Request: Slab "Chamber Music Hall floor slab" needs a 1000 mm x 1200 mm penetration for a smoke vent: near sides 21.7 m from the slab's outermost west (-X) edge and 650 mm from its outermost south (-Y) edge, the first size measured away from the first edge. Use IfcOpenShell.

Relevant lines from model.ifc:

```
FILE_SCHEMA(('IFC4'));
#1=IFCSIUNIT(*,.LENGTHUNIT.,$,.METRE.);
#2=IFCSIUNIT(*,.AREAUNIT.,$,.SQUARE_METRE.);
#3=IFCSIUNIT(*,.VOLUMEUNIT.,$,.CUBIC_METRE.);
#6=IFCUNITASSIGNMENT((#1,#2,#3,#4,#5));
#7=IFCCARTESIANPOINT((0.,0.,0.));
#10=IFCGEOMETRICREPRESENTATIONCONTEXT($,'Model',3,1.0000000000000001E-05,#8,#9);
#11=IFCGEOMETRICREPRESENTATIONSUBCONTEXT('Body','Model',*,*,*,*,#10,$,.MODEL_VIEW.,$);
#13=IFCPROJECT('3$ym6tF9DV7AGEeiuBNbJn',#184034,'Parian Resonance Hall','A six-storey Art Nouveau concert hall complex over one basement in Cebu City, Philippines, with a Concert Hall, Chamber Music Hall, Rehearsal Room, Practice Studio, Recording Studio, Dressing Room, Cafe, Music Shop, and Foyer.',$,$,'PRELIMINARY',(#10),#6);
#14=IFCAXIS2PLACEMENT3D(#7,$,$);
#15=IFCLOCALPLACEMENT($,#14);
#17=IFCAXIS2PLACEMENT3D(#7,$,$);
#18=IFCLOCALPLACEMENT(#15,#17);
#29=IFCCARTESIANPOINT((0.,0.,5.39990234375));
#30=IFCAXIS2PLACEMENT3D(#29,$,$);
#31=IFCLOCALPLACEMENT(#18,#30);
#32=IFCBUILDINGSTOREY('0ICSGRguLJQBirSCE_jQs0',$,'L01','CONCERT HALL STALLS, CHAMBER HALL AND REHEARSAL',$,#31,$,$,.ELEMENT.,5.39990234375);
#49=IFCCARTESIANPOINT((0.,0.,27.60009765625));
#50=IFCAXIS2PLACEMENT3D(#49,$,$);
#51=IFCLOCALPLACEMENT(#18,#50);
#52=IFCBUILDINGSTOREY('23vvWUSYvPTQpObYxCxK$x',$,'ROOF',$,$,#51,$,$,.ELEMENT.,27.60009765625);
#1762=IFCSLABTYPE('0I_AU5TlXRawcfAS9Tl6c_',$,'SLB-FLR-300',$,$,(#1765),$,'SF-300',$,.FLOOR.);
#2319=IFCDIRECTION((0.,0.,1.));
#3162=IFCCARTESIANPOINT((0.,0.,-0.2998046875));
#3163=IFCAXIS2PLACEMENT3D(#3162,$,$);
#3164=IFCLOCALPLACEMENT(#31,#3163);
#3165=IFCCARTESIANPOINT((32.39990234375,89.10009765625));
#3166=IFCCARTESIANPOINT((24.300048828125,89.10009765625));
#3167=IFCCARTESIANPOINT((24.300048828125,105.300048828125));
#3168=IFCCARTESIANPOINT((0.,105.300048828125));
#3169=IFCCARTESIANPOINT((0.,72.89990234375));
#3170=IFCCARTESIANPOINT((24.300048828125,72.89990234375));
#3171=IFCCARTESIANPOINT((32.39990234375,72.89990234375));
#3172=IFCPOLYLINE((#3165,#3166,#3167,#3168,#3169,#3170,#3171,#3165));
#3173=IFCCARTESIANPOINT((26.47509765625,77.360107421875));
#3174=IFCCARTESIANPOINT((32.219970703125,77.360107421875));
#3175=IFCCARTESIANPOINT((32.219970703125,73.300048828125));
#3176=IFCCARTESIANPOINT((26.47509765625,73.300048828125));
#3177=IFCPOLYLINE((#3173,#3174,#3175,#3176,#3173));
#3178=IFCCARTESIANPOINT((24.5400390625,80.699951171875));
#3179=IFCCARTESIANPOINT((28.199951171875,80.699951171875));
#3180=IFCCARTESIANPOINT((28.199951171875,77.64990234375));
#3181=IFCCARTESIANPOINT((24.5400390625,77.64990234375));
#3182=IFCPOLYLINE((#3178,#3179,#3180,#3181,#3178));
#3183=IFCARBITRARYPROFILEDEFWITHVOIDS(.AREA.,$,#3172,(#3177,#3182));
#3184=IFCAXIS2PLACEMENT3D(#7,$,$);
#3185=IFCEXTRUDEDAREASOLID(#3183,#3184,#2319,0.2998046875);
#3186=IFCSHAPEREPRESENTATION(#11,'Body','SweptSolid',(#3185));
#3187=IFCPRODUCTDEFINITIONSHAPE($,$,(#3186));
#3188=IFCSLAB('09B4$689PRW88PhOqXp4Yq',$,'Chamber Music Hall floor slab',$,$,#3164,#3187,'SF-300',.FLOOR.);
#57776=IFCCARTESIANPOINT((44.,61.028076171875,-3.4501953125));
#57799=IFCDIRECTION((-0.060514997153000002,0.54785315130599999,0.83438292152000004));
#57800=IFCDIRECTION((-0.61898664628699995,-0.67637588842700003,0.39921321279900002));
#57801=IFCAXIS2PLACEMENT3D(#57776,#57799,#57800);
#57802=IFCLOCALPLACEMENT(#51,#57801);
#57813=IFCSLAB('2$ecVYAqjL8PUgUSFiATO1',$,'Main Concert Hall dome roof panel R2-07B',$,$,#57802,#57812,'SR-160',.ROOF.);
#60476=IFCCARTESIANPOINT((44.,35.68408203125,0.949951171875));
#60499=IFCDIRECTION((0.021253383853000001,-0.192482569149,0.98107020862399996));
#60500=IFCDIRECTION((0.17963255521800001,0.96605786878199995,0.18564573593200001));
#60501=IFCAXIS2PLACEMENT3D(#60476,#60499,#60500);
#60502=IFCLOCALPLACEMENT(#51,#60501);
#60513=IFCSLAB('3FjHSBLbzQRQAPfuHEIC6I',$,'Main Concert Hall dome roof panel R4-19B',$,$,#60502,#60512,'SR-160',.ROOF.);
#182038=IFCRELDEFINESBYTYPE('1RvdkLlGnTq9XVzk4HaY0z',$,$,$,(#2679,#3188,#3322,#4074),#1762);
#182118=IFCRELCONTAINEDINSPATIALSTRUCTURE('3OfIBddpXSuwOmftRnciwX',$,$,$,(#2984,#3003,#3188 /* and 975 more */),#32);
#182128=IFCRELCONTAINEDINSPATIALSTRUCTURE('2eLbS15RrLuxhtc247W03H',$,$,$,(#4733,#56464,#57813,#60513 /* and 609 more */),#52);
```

```python
import numpy as np
import ifcopenshell
import ifcopenshell.api.feature
import ifcopenshell.api.geometry
import ifcopenshell.api.root
import ifcopenshell.geom
import ifcopenshell.util.placement
import ifcopenshell.util.representation
import ifcopenshell.util.shape
import ifcopenshell.util.unit

model = ifcopenshell.open("model.ifc")
unit_scale = ifcopenshell.util.unit.calculate_unit_scale(model)
settings = ifcopenshell.geom.settings()


def volume(element):
    """Net volume in cubic metres, openings subtracted."""
    shape = ifcopenshell.geom.create_shape(settings, element)
    return ifcopenshell.util.shape.get_volume(shape.geometry)


slab = model.by_guid("09B4$689PRW88PhOqXp4Yq")
before = volume(slab)

# Extent in the slab's own axes, in metres. The edges named are its -X and -Y sides.
slab_shape = ifcopenshell.geom.create_shape(settings, slab)
vertices = ifcopenshell.util.shape.get_vertices(slab_shape.geometry)
x_min, y_min, bottom = vertices.min(axis=0)
top = vertices[:, 2].max()

opening = ifcopenshell.api.root.create_entity(model, ifc_class="IfcOpeningElement", name="Smoke vent opening", predefined_type="OPENING")
context = ifcopenshell.util.representation.get_context(model, "Model", "Body", "MODEL_VIEW")
width, depth = 1, 1.2
outline = [(0.0, 0.0), (width, 0.0), (width, depth), (0.0, depth), (0.0, 0.0)]
# Overshoot both faces by 50 mm so the cut is clean.
shape = ifcopenshell.api.geometry.add_slab_representation(
    model, context=context, depth=top - bottom + 0.1, polyline=outline
)
ifcopenshell.api.geometry.assign_representation(model, product=opening, representation=shape)

matrix = ifcopenshell.util.placement.get_local_placement(slab.ObjectPlacement)
matrix[:, 3] = matrix @ np.append(np.array([x_min + 21.7, y_min + 0.65, bottom - 0.05]) / unit_scale, 1.0)
ifcopenshell.api.geometry.edit_object_placement(model, product=opening, matrix=matrix, is_si=False)
ifcopenshell.api.feature.add_feature(model, feature=opening, element=slab)

after = volume(slab)

print(f"slab volume {before:.3f} -> {after:.3f} m3")

model.write("model_updated.ifc")
```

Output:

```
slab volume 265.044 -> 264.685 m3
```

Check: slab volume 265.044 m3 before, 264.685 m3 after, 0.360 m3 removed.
